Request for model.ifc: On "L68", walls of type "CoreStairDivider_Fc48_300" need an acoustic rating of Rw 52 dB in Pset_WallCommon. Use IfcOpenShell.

First a look at what the model holds.

```python
import ifcopenshell
import ifcopenshell.util.element

model = ifcopenshell.open("model.ifc")
print(model.schema)
storey = next(s for s in model.by_type("IfcBuildingStorey") if s.Name == "L68")
walls = [e for e in ifcopenshell.util.element.get_decomposition(storey) if e.is_a("IfcWall")]
seen = {}
for e in walls:
    element_type = ifcopenshell.util.element.get_type(e)
    key = (element_type.Name if element_type != e and element_type else None, ifcopenshell.util.element.get_pset(e, "Pset_WallCommon", "AcousticRating"))
    seen[key] = seen.get(key, 0) + 1
for (name, value), count in sorted(seen.items(), key=str):
    print(count, "x", name, "|", value)
```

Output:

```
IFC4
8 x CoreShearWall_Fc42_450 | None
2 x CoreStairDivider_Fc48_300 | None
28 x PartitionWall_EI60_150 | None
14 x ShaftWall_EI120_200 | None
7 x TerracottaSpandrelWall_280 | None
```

```python
import ifcopenshell
import ifcopenshell.api.pset
import ifcopenshell.util.element

model = ifcopenshell.open("model.ifc")

storey = next(s for s in model.by_type("IfcBuildingStorey") if s.Name == "L68")
walls = [e for e in ifcopenshell.util.element.get_decomposition(storey) if e.is_a("IfcWall")]

count = 0
for e in walls:
    element_type = ifcopenshell.util.element.get_type(e)
    if element_type in (None, e) or element_type.Name != "CoreStairDivider_Fc48_300":
        continue
    # add_pset returns the element's existing set when there is one.
    pset = ifcopenshell.api.pset.add_pset(model, product=e, name="Pset_WallCommon")
    ifcopenshell.api.pset.edit_pset(model, pset=pset, properties={"AcousticRating": "Rw 52 dB"})
    count += 1

print(count, "walls updated")

model.write("model_updated.ifc")
```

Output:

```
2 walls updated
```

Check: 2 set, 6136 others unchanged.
